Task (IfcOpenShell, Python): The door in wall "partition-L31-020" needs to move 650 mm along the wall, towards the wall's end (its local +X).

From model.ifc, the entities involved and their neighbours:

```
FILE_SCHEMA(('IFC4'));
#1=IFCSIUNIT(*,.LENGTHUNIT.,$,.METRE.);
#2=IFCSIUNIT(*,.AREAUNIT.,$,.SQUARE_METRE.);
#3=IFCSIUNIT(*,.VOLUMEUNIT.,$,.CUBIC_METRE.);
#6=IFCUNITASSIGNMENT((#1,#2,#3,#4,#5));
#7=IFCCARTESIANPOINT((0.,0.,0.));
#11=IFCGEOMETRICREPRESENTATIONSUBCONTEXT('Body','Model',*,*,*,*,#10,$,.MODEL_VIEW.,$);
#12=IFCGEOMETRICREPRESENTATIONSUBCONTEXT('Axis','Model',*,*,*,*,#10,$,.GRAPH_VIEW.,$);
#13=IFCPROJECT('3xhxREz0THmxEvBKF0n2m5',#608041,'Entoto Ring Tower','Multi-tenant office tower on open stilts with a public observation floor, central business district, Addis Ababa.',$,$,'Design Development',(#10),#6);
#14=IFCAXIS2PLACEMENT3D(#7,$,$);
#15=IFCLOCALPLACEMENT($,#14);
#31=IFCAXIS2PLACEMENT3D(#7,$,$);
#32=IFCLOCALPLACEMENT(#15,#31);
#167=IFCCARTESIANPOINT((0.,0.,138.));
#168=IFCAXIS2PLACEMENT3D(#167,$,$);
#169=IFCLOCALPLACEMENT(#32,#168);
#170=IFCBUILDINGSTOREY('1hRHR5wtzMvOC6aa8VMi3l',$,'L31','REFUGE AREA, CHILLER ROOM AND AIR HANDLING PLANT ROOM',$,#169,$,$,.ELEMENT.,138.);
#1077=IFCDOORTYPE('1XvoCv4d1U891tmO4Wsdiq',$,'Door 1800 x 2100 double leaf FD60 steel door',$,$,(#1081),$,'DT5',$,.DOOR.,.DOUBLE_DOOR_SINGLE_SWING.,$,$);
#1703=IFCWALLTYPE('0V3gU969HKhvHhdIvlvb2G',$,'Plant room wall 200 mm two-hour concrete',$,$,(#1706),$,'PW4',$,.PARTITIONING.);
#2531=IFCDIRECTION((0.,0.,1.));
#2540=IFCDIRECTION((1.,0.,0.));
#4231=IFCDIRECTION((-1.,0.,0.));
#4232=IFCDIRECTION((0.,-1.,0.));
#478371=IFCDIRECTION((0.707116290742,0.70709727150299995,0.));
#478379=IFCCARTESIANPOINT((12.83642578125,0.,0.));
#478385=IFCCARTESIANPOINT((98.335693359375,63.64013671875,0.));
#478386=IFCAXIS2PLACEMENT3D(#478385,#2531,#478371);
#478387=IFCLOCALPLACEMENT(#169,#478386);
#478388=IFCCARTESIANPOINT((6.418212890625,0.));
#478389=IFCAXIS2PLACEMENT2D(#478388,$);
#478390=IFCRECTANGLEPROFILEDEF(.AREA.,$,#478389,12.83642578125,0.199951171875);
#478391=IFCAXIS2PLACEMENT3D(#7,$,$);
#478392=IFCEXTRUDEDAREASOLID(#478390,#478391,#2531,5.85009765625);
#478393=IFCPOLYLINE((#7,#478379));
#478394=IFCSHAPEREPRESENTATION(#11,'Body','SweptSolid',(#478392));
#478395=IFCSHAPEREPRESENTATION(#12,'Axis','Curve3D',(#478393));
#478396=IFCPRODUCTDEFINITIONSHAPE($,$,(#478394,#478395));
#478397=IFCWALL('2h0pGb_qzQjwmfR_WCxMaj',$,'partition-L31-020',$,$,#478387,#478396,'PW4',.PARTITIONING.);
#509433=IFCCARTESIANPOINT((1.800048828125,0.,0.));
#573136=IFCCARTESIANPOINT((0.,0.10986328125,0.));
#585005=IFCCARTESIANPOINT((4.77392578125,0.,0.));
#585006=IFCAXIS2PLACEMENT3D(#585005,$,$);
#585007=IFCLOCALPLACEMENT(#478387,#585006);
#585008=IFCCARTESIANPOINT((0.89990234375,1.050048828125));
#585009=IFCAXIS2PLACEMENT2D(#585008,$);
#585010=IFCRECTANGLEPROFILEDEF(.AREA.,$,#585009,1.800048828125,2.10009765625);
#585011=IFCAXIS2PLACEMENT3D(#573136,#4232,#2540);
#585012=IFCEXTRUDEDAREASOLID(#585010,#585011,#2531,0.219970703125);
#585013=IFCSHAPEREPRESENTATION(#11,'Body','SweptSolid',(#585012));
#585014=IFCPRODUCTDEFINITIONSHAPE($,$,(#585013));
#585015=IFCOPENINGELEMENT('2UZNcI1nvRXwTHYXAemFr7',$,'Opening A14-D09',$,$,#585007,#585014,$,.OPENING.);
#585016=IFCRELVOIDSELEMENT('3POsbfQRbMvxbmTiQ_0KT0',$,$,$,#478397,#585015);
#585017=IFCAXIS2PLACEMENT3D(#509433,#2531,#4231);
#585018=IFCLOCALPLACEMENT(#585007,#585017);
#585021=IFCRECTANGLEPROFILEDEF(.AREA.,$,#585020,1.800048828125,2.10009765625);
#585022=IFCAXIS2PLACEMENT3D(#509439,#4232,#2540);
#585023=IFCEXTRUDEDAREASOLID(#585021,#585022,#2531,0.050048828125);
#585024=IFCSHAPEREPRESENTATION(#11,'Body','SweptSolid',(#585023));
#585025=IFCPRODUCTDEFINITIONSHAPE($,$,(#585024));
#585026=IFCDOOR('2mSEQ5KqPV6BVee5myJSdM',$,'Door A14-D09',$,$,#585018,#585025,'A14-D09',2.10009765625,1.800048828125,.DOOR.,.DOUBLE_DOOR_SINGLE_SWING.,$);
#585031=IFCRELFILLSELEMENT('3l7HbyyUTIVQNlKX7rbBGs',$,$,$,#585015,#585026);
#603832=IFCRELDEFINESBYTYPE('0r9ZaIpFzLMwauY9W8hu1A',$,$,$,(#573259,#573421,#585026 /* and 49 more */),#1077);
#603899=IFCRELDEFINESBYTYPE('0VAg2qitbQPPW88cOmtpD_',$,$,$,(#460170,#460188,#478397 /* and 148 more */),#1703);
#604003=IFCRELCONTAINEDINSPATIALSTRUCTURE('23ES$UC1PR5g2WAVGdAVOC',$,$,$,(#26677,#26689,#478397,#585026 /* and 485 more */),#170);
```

```python
import ifcopenshell
import ifcopenshell.api.geometry
import ifcopenshell.util.placement
import ifcopenshell.util.unit

model = ifcopenshell.open("model.ifc")
unit_scale = ifcopenshell.util.unit.calculate_unit_scale(model)

door = model.by_guid("2mSEQ5KqPV6BVee5myJSdM")
opening = door.FillsVoids[0].RelatingOpeningElement
wall = opening.VoidsElements[0].RelatingBuildingElement

wall_matrix = ifcopenshell.util.placement.get_local_placement(wall.ObjectPlacement)
shift = wall_matrix[:3, 0] * 0.65 / unit_scale
before = ifcopenshell.util.placement.get_local_placement(door.ObjectPlacement)[:3, 3].copy()

# The door is placed relative to its opening, so it follows when the opening moves.
matrix = ifcopenshell.util.placement.get_local_placement(opening.ObjectPlacement)
matrix[:3, 3] += shift
ifcopenshell.api.geometry.edit_object_placement(
    model, product=opening, matrix=matrix, is_si=False, should_transform_children=True
)

after = ifcopenshell.util.placement.get_local_placement(door.ObjectPlacement)[:3, 3]
print("door moved by", (after - before).round(3) + 0.0)

model.write("model_edited.ifc")
```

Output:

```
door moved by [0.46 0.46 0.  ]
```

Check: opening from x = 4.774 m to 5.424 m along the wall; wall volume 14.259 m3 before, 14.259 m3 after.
